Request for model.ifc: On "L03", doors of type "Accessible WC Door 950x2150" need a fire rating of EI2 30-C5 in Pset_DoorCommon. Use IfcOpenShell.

First a look at what the model holds.

```python
import ifcopenshell
import ifcopenshell.util.element

model = ifcopenshell.open("model.ifc")
print(model.schema)
storey = next(s for s in model.by_type("IfcBuildingStorey") if s.Name == "L03")
doors = [e for e in ifcopenshell.util.element.get_decomposition(storey) if e.is_a("IfcDoor")]
seen = {}
for e in doors:
    element_type = ifcopenshell.util.element.get_type(e)
    key = (element_type.Name if element_type != e and element_type else None, ifcopenshell.util.element.get_pset(e, "Pset_DoorCommon", "FireRating"))
    seen[key] = seen.get(key, 0) + 1
for (name, value), count in sorted(seen.items(), key=str):
    print(count, "x", name, "|", value)
```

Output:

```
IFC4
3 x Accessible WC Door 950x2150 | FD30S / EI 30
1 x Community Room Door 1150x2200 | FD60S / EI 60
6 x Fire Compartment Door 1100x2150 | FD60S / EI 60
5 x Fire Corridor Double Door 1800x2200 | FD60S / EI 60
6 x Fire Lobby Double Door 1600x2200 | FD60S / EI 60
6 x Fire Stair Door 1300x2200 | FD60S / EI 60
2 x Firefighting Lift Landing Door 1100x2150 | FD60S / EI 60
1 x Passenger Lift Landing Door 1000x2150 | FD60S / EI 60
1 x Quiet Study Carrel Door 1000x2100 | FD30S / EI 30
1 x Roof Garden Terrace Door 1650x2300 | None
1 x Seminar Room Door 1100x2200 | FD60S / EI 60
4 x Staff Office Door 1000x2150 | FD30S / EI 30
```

```python
import ifcopenshell
import ifcopenshell.api.pset
import ifcopenshell.util.element

model = ifcopenshell.open("model.ifc")

storey = next(s for s in model.by_type("IfcBuildingStorey") if s.Name == "L03")
doors = [e for e in ifcopenshell.util.element.get_decomposition(storey) if e.is_a("IfcDoor")]

count = 0
for e in doors:
    element_type = ifcopenshell.util.element.get_type(e)
    if element_type in (None, e) or element_type.Name != "Accessible WC Door 950x2150":
        continue
    # add_pset returns the element's existing set when there is one.
    pset = ifcopenshell.api.pset.add_pset(model, product=e, name="Pset_DoorCommon")
    ifcopenshell.api.pset.edit_pset(model, pset=pset, properties={"FireRating": "EI2 30-C5"})
    count += 1

print(count, "doors updated")

model.write("model_v2.ifc")
```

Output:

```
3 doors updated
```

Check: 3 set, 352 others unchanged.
